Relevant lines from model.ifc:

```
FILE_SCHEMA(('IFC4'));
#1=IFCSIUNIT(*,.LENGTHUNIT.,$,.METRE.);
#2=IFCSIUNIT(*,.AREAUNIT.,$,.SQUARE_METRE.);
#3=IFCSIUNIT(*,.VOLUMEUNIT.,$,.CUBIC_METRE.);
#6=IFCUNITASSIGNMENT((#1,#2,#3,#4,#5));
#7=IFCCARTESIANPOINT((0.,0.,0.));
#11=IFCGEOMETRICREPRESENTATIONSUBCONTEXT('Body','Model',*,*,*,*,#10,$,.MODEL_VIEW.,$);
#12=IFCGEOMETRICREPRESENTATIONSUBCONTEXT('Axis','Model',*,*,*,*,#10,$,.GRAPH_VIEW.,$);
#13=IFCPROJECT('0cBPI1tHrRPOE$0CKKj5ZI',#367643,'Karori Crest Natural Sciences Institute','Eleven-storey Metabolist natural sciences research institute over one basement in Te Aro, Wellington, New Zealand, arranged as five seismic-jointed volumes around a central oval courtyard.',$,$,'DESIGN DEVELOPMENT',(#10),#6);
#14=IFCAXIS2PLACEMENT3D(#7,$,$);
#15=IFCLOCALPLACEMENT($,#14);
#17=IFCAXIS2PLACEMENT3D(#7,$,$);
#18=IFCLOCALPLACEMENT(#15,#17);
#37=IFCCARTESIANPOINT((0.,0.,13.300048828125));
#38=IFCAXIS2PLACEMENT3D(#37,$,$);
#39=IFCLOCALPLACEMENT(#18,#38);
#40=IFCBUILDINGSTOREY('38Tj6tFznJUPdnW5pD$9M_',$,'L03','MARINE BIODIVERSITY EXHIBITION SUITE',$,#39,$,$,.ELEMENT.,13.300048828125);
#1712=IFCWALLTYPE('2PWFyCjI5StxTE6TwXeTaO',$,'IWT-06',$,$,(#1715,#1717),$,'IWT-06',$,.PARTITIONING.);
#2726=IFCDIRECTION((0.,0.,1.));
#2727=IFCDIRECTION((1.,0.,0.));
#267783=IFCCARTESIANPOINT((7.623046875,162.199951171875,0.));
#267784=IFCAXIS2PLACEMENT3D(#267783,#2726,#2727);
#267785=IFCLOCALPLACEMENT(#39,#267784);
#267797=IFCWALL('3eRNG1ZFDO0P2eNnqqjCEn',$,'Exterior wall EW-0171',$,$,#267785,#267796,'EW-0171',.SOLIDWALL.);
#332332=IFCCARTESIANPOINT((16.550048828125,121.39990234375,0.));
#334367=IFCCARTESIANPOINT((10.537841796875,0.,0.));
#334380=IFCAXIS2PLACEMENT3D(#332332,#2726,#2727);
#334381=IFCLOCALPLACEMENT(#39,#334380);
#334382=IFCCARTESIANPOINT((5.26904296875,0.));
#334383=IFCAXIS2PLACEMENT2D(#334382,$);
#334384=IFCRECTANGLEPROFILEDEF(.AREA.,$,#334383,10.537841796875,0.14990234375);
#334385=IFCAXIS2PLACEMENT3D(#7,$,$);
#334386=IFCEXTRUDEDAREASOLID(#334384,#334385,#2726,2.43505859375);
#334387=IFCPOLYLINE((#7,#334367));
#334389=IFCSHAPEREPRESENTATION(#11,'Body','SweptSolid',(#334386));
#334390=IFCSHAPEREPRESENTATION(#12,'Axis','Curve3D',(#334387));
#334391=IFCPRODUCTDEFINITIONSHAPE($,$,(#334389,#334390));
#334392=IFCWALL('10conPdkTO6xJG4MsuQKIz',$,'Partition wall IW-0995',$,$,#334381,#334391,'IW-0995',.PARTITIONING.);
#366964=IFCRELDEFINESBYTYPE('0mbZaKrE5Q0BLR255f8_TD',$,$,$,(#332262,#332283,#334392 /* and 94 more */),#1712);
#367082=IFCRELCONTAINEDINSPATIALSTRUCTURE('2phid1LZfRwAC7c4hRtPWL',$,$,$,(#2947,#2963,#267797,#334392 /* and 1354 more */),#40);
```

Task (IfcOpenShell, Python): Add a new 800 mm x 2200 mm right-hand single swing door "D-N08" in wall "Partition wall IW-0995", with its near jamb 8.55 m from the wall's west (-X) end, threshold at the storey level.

```python
import numpy as np
import ifcopenshell
import ifcopenshell.api.feature
import ifcopenshell.api.geometry
import ifcopenshell.api.root
import ifcopenshell.api.spatial
import ifcopenshell.geom
import ifcopenshell.util.element
import ifcopenshell.util.placement
import ifcopenshell.util.representation
import ifcopenshell.util.shape
import ifcopenshell.util.unit

model = ifcopenshell.open("model.ifc")
unit_scale = ifcopenshell.util.unit.calculate_unit_scale(model)
settings = ifcopenshell.geom.settings()


def volume(element):
    """Net volume in cubic metres, openings subtracted."""
    shape = ifcopenshell.geom.create_shape(settings, element)
    return ifcopenshell.util.shape.get_volume(shape.geometry)


wall = model.by_guid("10conPdkTO6xJG4MsuQKIz")
storey = ifcopenshell.util.element.get_container(wall, ifc_class="IfcBuildingStorey")
context = ifcopenshell.util.representation.get_context(model, "Model", "Body", "MODEL_VIEW")
before = volume(wall)

width, height, from_end, sill = 0.8, 2.2, 8.55, 0.0  # metres

# The wall runs along its own X axis, and the end named is its -X end.
wall_shape = ifcopenshell.geom.create_shape(settings, wall)
x, y, z = ifcopenshell.util.shape.get_vertices(wall_shape.geometry).T
start = x.min() + from_end
face, thickness = float(y.min()), float(y.max() - y.min())
wall_matrix = ifcopenshell.util.placement.get_local_placement(wall.ObjectPlacement)
level = ifcopenshell.util.placement.get_local_placement(storey.ObjectPlacement)[2, 3]


def in_wall(x, y):
    """Placement at x, y metres in the wall's axes, at sill height."""
    matrix = wall_matrix.copy()
    matrix[:, 3] = wall_matrix @ np.array([x / unit_scale, y / unit_scale, 0.0, 1.0])
    matrix[2, 3] = level + sill / unit_scale
    return matrix


# Opening: a box that overshoots both wall faces by 50 mm.
opening = ifcopenshell.api.root.create_entity(model, ifc_class="IfcOpeningElement", predefined_type="OPENING")
box = ifcopenshell.api.geometry.add_wall_representation(
    model, context=context, length=width, height=height, thickness=thickness + 0.1
)
ifcopenshell.api.geometry.assign_representation(model, product=opening, representation=box)
ifcopenshell.api.geometry.edit_object_placement(model, product=opening, matrix=in_wall(start, face - 0.05), is_si=False)
ifcopenshell.api.feature.add_feature(model, feature=opening, element=wall)

door = ifcopenshell.api.root.create_entity(model, ifc_class="IfcDoor", name="D-N08", predefined_type="DOOR")
door.OverallWidth, door.OverallHeight = width / unit_scale, height / unit_scale
door.OperationType = "SINGLE_SWING_RIGHT"
body = ifcopenshell.api.geometry.add_door_representation(
    model,
    context=context,
    overall_width=door.OverallWidth,
    overall_height=door.OverallHeight,
    operation_type="SINGLE_SWING_RIGHT",
    lining_properties={"LiningDepth": thickness / unit_scale, "ThresholdDepth": thickness / unit_scale},
)
ifcopenshell.api.geometry.assign_representation(model, product=door, representation=body)
ifcopenshell.api.spatial.assign_container(model, products=[door], relating_structure=storey)
ifcopenshell.api.feature.add_filling(model, opening=opening, element=door)

# The lining spans the wall, so the door starts at the wall face.
ifcopenshell.api.geometry.edit_object_placement(model, product=door, matrix=in_wall(start, face), is_si=False)

after = volume(wall)

print(f"wall volume {before:.3f} -> {after:.3f} m3")

model.write("model_updated.ifc")
```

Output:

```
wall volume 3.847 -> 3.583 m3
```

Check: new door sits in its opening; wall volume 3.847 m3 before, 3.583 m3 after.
